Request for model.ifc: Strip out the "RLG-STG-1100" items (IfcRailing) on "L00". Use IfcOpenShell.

First a look at what the model holds.

```python
import ifcopenshell
import ifcopenshell.util.element

model = ifcopenshell.open("model.ifc")
print(model.schema)
storey = next(s for s in model.by_type("IfcBuildingStorey") if s.Name == "L00")
railings = [e for e in ifcopenshell.util.element.get_decomposition(storey) if e.is_a("IfcRailing")]
seen = {}
for e in railings:
    element_type = ifcopenshell.util.element.get_type(e)
    name = element_type.Name if element_type not in (None, e) else None
    seen[name] = seen.get(name, 0) + 1
for name, count in sorted(seen.items(), key=str):
    print(count, "x", name)
```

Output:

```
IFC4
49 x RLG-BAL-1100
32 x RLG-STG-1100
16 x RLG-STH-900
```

```python
import ifcopenshell
import ifcopenshell.api.root
import ifcopenshell.util.element

model = ifcopenshell.open("model.ifc")

storey = next(s for s in model.by_type("IfcBuildingStorey") if s.Name == "L00")
railings = [e for e in ifcopenshell.util.element.get_decomposition(storey) if e.is_a("IfcRailing")]
targets = [e for e in railings if (t := ifcopenshell.util.element.get_type(e)) not in (None, e) and t.Name == "RLG-STG-1100"]

for e in targets:
    ifcopenshell.api.root.remove_product(model, product=e)
print(len(targets), "removed")

model.write("model_edited.ifc")
```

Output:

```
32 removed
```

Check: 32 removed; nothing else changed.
